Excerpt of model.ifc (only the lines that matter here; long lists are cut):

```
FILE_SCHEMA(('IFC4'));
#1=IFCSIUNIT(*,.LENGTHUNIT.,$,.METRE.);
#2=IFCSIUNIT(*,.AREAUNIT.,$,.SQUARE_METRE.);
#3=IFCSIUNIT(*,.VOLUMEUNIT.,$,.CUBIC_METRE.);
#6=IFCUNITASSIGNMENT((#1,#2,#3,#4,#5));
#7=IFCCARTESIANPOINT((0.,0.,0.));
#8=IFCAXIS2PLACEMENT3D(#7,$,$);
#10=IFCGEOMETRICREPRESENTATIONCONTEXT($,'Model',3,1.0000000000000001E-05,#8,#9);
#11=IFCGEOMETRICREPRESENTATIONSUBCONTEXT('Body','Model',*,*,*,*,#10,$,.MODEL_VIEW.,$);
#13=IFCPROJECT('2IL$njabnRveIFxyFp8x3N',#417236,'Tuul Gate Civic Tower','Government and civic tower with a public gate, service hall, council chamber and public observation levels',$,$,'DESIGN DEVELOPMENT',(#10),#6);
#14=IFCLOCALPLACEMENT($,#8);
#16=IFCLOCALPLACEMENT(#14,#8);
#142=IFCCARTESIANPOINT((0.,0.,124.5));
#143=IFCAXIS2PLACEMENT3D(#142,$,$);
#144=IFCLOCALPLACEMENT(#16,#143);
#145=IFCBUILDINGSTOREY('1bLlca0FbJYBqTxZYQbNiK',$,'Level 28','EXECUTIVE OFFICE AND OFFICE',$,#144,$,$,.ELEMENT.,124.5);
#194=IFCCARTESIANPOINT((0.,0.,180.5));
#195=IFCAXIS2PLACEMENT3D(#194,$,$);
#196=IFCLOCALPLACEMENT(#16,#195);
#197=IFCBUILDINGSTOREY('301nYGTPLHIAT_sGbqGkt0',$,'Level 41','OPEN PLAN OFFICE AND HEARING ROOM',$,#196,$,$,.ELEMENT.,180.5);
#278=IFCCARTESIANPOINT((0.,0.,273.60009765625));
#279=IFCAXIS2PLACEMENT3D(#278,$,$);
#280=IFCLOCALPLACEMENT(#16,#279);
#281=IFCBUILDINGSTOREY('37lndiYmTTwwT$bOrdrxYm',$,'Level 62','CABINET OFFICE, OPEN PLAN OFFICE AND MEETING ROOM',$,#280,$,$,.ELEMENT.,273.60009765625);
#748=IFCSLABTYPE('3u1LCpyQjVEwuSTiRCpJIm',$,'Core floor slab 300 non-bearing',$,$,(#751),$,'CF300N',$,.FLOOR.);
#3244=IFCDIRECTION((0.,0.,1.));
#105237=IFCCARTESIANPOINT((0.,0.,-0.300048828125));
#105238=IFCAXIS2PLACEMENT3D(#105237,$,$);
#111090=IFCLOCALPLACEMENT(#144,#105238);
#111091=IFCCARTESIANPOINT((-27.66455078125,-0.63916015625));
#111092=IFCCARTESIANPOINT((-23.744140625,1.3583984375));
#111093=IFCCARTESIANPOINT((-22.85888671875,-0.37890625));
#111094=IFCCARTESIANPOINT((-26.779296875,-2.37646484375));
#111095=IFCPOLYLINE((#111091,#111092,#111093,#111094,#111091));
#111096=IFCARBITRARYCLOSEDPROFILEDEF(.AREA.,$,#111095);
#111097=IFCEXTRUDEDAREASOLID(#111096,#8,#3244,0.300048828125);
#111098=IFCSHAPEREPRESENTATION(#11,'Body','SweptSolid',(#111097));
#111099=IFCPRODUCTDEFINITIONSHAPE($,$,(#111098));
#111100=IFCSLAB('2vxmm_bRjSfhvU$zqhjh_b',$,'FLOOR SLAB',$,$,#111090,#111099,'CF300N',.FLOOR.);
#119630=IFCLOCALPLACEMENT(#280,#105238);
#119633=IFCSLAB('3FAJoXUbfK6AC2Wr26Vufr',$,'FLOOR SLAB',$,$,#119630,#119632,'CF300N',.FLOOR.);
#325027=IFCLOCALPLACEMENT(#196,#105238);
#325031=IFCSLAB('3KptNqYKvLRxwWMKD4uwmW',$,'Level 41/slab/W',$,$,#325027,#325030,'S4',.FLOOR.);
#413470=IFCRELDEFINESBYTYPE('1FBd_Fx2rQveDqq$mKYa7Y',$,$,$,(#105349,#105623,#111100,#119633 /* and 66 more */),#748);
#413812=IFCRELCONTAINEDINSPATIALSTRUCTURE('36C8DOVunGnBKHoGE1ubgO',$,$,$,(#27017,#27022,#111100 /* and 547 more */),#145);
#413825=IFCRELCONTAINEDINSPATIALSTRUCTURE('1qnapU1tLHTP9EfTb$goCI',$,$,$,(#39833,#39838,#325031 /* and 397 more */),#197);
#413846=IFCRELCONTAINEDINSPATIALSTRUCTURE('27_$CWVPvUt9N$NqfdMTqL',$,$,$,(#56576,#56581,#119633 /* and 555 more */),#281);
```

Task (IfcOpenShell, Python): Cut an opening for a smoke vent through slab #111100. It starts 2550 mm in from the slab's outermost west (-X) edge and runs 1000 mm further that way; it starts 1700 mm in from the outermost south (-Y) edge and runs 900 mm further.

```python
import numpy as np
import ifcopenshell
import ifcopenshell.api.feature
import ifcopenshell.api.geometry
import ifcopenshell.api.root
import ifcopenshell.geom
import ifcopenshell.util.placement
import ifcopenshell.util.representation
import ifcopenshell.util.shape
import ifcopenshell.util.unit

model = ifcopenshell.open("model.ifc")
unit_scale = ifcopenshell.util.unit.calculate_unit_scale(model)
settings = ifcopenshell.geom.settings()


def volume(element):
    """Net volume in cubic metres, openings subtracted."""
    shape = ifcopenshell.geom.create_shape(settings, element)
    return ifcopenshell.util.shape.get_volume(shape.geometry)


slab = model.by_guid("2vxmm_bRjSfhvU$zqhjh_b")
before = volume(slab)

# Extent in the slab's own axes, in metres. The edges named are its -X and -Y sides.
slab_shape = ifcopenshell.geom.create_shape(settings, slab)
vertices = ifcopenshell.util.shape.get_vertices(slab_shape.geometry)
x_min, y_min, bottom = vertices.min(axis=0)
top = vertices[:, 2].max()

opening = ifcopenshell.api.root.create_entity(model, ifc_class="IfcOpeningElement", name="Smoke vent opening", predefined_type="OPENING")
context = ifcopenshell.util.representation.get_context(model, "Model", "Body", "MODEL_VIEW")
width, depth = 1, 0.9
outline = [(0.0, 0.0), (width, 0.0), (width, depth), (0.0, depth), (0.0, 0.0)]
# Overshoot both faces by 50 mm so the cut is clean.
shape = ifcopenshell.api.geometry.add_slab_representation(
    model, context=context, depth=top - bottom + 0.1, polyline=outline
)
ifcopenshell.api.geometry.assign_representation(model, product=opening, representation=shape)

matrix = ifcopenshell.util.placement.get_local_placement(slab.ObjectPlacement)
matrix[:, 3] = matrix @ np.append(np.array([x_min + 2.55, y_min + 1.7, bottom - 0.05]) / unit_scale, 1.0)
ifcopenshell.api.geometry.edit_object_placement(model, product=opening, matrix=matrix, is_si=False)
ifcopenshell.api.feature.add_feature(model, feature=opening, element=slab)

after = volume(slab)

print(f"slab volume {before:.3f} -> {after:.3f} m3")

model.write("model_rev.ifc")
```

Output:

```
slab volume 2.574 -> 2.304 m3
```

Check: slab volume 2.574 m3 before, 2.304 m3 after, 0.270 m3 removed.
